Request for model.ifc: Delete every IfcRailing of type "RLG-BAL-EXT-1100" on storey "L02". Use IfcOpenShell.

First a look at what the model holds.

```python
import ifcopenshell
import ifcopenshell.util.element

model = ifcopenshell.open("model.ifc")
print(model.schema)
storey = next(s for s in model.by_type("IfcBuildingStorey") if s.Name == "L02")
railings = [e for e in ifcopenshell.util.element.get_decomposition(storey) if e.is_a("IfcRailing")]
seen = {}
for e in railings:
    element_type = ifcopenshell.util.element.get_type(e)
    name = element_type.Name if element_type not in (None, e) else None
    seen[name] = seen.get(name, 0) + 1
for name, count in sorted(seen.items(), key=str):
    print(count, "x", name)
```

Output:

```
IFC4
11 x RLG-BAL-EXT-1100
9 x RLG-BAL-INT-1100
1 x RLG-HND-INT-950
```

```python
import ifcopenshell
import ifcopenshell.api.root
import ifcopenshell.util.element

model = ifcopenshell.open("model.ifc")

storey = next(s for s in model.by_type("IfcBuildingStorey") if s.Name == "L02")
railings = [e for e in ifcopenshell.util.element.get_decomposition(storey) if e.is_a("IfcRailing")]
targets = [e for e in railings if (t := ifcopenshell.util.element.get_type(e)) not in (None, e) and t.Name == "RLG-BAL-EXT-1100"]

for e in targets:
    ifcopenshell.api.root.remove_product(model, product=e)
print(len(targets), "removed")

model.write("model_updated.ifc")
```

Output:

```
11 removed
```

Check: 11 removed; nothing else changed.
